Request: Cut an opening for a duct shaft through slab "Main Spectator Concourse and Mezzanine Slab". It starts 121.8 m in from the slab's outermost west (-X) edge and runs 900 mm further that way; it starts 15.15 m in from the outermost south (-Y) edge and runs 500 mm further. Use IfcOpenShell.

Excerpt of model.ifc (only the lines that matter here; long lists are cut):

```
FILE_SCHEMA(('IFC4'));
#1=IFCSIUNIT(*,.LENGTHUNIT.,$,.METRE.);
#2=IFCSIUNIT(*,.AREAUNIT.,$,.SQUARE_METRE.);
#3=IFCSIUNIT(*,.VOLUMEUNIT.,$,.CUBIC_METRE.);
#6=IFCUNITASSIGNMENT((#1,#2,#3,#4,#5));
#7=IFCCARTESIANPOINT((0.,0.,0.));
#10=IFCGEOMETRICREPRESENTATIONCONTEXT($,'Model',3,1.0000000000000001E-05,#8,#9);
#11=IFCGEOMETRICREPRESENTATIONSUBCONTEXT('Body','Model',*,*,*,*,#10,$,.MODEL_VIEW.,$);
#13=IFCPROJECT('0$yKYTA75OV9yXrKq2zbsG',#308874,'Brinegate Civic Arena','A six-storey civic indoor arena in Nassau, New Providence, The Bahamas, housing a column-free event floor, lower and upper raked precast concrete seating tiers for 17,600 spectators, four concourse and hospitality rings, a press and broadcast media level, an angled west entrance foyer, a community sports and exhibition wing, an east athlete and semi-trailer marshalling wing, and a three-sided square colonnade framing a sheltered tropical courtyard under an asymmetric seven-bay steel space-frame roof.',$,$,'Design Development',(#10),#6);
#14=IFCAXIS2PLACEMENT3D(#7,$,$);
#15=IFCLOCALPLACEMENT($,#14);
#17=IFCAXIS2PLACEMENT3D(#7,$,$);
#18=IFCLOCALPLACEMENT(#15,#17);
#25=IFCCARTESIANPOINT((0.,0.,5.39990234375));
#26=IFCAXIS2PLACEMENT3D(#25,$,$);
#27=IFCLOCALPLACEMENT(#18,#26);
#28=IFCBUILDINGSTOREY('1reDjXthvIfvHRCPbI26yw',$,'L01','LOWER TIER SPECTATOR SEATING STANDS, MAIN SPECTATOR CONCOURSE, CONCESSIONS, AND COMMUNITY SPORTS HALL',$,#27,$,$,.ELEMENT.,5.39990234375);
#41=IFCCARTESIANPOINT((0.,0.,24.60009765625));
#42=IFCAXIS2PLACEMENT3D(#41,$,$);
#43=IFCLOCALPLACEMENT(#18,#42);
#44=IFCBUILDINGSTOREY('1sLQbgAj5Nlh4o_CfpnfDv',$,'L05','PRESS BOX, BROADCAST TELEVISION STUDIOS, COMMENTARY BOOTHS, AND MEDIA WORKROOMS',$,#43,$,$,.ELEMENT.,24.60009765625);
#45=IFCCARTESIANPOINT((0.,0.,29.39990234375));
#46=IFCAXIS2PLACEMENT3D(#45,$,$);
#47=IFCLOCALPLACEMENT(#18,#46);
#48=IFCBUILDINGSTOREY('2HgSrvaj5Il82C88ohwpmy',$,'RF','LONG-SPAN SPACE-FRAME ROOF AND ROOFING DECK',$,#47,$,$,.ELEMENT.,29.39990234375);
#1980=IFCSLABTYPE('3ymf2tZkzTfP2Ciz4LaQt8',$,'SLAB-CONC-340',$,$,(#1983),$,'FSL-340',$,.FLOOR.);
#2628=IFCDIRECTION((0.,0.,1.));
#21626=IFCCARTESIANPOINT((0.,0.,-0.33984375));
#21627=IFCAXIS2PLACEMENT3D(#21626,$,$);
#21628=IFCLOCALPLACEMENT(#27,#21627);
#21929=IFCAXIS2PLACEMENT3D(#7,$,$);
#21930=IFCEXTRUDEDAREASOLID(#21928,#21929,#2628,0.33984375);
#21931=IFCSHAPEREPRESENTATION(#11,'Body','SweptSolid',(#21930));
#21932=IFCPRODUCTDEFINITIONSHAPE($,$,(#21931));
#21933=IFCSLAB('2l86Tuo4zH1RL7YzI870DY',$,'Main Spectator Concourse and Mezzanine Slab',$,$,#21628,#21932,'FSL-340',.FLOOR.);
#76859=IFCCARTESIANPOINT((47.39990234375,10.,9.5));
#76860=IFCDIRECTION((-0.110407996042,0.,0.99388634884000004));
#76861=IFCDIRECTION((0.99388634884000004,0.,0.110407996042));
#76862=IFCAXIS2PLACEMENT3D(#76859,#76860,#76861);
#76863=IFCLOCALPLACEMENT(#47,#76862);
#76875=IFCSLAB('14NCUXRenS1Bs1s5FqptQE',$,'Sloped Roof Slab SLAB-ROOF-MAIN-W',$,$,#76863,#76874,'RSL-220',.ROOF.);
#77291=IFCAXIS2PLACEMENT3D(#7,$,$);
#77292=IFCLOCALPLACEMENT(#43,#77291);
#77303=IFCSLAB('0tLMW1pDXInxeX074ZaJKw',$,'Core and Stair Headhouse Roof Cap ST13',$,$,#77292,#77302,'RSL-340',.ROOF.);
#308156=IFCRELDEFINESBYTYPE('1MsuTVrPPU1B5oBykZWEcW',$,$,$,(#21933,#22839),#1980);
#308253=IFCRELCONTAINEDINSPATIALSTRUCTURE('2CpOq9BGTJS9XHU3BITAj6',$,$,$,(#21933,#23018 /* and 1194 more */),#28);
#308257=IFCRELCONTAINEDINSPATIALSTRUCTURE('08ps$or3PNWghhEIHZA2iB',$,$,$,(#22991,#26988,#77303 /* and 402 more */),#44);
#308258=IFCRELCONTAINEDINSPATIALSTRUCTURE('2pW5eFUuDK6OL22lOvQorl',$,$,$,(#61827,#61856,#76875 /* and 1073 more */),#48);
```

```python
import numpy as np
import ifcopenshell
import ifcopenshell.api.feature
import ifcopenshell.api.geometry
import ifcopenshell.api.root
import ifcopenshell.geom
import ifcopenshell.util.placement
import ifcopenshell.util.representation
import ifcopenshell.util.shape
import ifcopenshell.util.unit

model = ifcopenshell.open("model.ifc")
unit_scale = ifcopenshell.util.unit.calculate_unit_scale(model)
settings = ifcopenshell.geom.settings()


def volume(element):
    """Net volume in cubic metres, openings subtracted."""
    shape = ifcopenshell.geom.create_shape(settings, element)
    return ifcopenshell.util.shape.get_volume(shape.geometry)


slab = model.by_guid("2l86Tuo4zH1RL7YzI870DY")
before = volume(slab)

# Extent in the slab's own axes, in metres. The edges named are its -X and -Y sides.
slab_shape = ifcopenshell.geom.create_shape(settings, slab)
vertices = ifcopenshell.util.shape.get_vertices(slab_shape.geometry)
x_min, y_min, bottom = vertices.min(axis=0)
top = vertices[:, 2].max()

opening = ifcopenshell.api.root.create_entity(model, ifc_class="IfcOpeningElement", name="Duct shaft opening", predefined_type="OPENING")
context = ifcopenshell.util.representation.get_context(model, "Model", "Body", "MODEL_VIEW")
width, depth = 0.9, 0.5
outline = [(0.0, 0.0), (width, 0.0), (width, depth), (0.0, depth), (0.0, 0.0)]
# Overshoot both faces by 50 mm so the cut is clean.
shape = ifcopenshell.api.geometry.add_slab_representation(
    model, context=context, depth=top - bottom + 0.1, polyline=outline
)
ifcopenshell.api.geometry.assign_representation(model, product=opening, representation=shape)

matrix = ifcopenshell.util.placement.get_local_placement(slab.ObjectPlacement)
matrix[:, 3] = matrix @ np.append(np.array([x_min + 121.8, y_min + 15.15, bottom - 0.05]) / unit_scale, 1.0)
ifcopenshell.api.geometry.edit_object_placement(model, product=opening, matrix=matrix, is_si=False)
ifcopenshell.api.feature.add_feature(model, feature=opening, element=slab)

after = volume(slab)

print(f"slab volume {before:.3f} -> {after:.3f} m3")

model.write("model-out.ifc")
```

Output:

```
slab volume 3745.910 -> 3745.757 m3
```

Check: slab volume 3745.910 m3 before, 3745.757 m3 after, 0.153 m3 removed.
